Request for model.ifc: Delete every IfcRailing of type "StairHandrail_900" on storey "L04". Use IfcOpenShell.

First a look at what the model holds.

```python
import ifcopenshell
import ifcopenshell.util.element

model = ifcopenshell.open("model.ifc")
print(model.schema)
storey = next(s for s in model.by_type("IfcBuildingStorey") if s.Name == "L04")
railings = [e for e in ifcopenshell.util.element.get_decomposition(storey) if e.is_a("IfcRailing")]
seen = {}
for e in railings:
    element_type = ifcopenshell.util.element.get_type(e)
    name = element_type.Name if element_type not in (None, e) else None
    seen[name] = seen.get(name, 0) + 1
for name, count in sorted(seen.items(), key=str):
    print(count, "x", name)
```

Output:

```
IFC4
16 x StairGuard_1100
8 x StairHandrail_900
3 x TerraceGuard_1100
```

```python
import ifcopenshell
import ifcopenshell.api.root
import ifcopenshell.util.element

model = ifcopenshell.open("model.ifc")

storey = next(s for s in model.by_type("IfcBuildingStorey") if s.Name == "L04")
railings = [e for e in ifcopenshell.util.element.get_decomposition(storey) if e.is_a("IfcRailing")]
targets = [e for e in railings if (t := ifcopenshell.util.element.get_type(e)) not in (None, e) and t.Name == "StairHandrail_900"]

for e in targets:
    ifcopenshell.api.root.remove_product(model, product=e)
print(len(targets), "removed")

model.write("model_edited.ifc")
```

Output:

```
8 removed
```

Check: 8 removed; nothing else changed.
